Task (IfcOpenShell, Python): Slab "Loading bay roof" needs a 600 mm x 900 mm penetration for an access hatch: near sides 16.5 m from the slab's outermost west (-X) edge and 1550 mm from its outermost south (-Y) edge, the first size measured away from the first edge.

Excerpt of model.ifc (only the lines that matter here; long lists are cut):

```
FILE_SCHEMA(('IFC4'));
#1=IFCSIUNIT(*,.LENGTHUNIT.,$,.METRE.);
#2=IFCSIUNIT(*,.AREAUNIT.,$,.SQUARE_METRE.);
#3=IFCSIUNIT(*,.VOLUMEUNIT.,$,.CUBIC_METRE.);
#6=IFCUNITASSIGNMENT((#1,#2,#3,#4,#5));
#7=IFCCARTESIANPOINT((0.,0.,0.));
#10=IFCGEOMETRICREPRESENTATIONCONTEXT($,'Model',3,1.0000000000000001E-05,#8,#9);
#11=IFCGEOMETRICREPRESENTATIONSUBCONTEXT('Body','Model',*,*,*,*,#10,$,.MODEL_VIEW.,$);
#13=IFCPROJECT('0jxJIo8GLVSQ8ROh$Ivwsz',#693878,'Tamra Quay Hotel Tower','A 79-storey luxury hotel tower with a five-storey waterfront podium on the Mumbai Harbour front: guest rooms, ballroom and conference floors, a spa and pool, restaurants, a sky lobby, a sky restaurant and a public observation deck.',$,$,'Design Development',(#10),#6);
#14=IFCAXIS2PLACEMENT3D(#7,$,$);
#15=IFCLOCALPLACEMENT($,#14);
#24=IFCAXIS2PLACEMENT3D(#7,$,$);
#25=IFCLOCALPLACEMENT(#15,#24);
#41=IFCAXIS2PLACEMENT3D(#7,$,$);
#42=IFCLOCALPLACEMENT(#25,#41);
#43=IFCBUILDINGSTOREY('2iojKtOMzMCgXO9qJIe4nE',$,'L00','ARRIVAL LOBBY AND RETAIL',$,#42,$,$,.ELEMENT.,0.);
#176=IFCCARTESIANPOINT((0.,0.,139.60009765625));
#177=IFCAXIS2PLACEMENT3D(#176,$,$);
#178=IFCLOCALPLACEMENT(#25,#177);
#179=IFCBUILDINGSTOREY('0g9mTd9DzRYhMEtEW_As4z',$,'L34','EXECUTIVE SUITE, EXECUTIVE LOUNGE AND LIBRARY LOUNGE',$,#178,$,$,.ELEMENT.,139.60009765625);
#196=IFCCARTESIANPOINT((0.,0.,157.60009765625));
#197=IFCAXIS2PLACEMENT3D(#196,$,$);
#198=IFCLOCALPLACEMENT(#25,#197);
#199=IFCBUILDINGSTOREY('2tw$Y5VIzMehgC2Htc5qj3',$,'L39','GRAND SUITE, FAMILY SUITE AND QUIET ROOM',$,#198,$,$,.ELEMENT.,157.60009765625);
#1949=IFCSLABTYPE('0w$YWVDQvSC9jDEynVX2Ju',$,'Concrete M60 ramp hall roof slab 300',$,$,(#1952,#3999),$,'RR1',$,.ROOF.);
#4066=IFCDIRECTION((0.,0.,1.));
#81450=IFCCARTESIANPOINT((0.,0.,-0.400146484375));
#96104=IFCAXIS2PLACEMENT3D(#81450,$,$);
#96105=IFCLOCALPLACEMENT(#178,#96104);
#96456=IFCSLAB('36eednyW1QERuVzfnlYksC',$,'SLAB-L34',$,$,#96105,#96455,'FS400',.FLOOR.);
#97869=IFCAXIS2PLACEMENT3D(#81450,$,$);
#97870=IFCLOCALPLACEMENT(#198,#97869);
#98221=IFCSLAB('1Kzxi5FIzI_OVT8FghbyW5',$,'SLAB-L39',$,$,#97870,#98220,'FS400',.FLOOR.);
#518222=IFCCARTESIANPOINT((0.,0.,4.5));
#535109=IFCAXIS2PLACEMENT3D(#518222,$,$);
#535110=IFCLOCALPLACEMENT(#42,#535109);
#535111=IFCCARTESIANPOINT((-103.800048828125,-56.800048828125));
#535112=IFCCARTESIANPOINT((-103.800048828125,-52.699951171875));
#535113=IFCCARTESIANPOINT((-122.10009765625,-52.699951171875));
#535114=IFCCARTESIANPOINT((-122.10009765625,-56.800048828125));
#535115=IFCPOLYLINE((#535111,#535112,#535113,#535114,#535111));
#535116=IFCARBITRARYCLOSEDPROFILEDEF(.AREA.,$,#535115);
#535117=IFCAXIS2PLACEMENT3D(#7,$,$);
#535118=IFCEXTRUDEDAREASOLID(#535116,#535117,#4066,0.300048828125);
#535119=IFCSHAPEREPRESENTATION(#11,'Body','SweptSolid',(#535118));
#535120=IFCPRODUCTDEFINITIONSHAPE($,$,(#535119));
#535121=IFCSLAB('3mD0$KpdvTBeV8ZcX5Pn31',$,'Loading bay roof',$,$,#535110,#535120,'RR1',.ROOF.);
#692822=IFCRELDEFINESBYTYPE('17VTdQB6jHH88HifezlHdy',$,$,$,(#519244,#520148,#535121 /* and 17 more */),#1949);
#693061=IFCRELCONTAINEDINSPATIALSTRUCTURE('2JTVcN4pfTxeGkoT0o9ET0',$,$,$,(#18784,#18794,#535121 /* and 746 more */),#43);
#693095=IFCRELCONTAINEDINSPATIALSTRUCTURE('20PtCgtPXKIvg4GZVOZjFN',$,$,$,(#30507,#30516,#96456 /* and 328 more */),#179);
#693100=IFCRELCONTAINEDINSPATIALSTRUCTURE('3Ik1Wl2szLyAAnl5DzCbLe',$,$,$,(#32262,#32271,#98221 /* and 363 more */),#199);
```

```python
import numpy as np
import ifcopenshell
import ifcopenshell.api.feature
import ifcopenshell.api.geometry
import ifcopenshell.api.root
import ifcopenshell.geom
import ifcopenshell.util.placement
import ifcopenshell.util.representation
import ifcopenshell.util.shape
import ifcopenshell.util.unit

model = ifcopenshell.open("model.ifc")
unit_scale = ifcopenshell.util.unit.calculate_unit_scale(model)
settings = ifcopenshell.geom.settings()


def volume(element):
    """Net volume in cubic metres, openings subtracted."""
    shape = ifcopenshell.geom.create_shape(settings, element)
    return ifcopenshell.util.shape.get_volume(shape.geometry)


slab = model.by_guid("3mD0$KpdvTBeV8ZcX5Pn31")
before = volume(slab)

# Extent in the slab's own axes, in metres. The edges named are its -X and -Y sides.
slab_shape = ifcopenshell.geom.create_shape(settings, slab)
vertices = ifcopenshell.util.shape.get_vertices(slab_shape.geometry)
x_min, y_min, bottom = vertices.min(axis=0)
top = vertices[:, 2].max()

opening = ifcopenshell.api.root.create_entity(model, ifc_class="IfcOpeningElement", name="Access hatch opening", predefined_type="OPENING")
context = ifcopenshell.util.representation.get_context(model, "Model", "Body", "MODEL_VIEW")
width, depth = 0.6, 0.9
outline = [(0.0, 0.0), (width, 0.0), (width, depth), (0.0, depth), (0.0, 0.0)]
# Overshoot both faces by 50 mm so the cut is clean.
shape = ifcopenshell.api.geometry.add_slab_representation(
    model, context=context, depth=top - bottom + 0.1, polyline=outline
)
ifcopenshell.api.geometry.assign_representation(model, product=opening, representation=shape)

matrix = ifcopenshell.util.placement.get_local_placement(slab.ObjectPlacement)
matrix[:, 3] = matrix @ np.append(np.array([x_min + 16.5, y_min + 1.55, bottom - 0.05]) / unit_scale, 1.0)
ifcopenshell.api.geometry.edit_object_placement(model, product=opening, matrix=matrix, is_si=False)
ifcopenshell.api.feature.add_feature(model, feature=opening, element=slab)

after = volume(slab)

print(f"slab volume {before:.3f} -> {after:.3f} m3")

model.write("model_edited.ifc")
```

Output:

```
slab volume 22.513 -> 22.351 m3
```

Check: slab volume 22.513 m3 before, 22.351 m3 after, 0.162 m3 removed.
